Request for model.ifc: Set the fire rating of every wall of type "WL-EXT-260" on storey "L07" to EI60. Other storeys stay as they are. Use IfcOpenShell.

First a look at what the model holds.

```python
import ifcopenshell
import ifcopenshell.util.element

model = ifcopenshell.open("model.ifc")
print(model.schema)
storey = next(s for s in model.by_type("IfcBuildingStorey") if s.Name == "L07")
walls = [e for e in ifcopenshell.util.element.get_decomposition(storey) if e.is_a("IfcWall")]
seen = {}
for e in walls:
    element_type = ifcopenshell.util.element.get_type(e)
    key = (element_type.Name if element_type != e and element_type else None, ifcopenshell.util.element.get_pset(e, "Pset_WallCommon", "FireRating"))
    seen[key] = seen.get(key, 0) + 1
for (name, value), count in sorted(seen.items(), key=str):
    print(count, "x", name, "|", value)
```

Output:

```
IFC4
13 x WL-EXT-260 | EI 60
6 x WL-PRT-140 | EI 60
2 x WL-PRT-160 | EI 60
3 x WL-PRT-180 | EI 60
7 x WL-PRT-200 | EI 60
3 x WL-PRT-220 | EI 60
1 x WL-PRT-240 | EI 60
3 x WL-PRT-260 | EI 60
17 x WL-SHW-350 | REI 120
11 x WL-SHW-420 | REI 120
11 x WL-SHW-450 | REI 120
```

```python
import ifcopenshell
import ifcopenshell.api.pset
import ifcopenshell.util.element

model = ifcopenshell.open("model.ifc")

storey = next(s for s in model.by_type("IfcBuildingStorey") if s.Name == "L07")
walls = [e for e in ifcopenshell.util.element.get_decomposition(storey) if e.is_a("IfcWall")]

count = 0
for e in walls:
    element_type = ifcopenshell.util.element.get_type(e)
    if element_type in (None, e) or element_type.Name != "WL-EXT-260":
        continue
    # add_pset returns the element's existing set when there is one.
    pset = ifcopenshell.api.pset.add_pset(model, product=e, name="Pset_WallCommon")
    ifcopenshell.api.pset.edit_pset(model, pset=pset, properties={"FireRating": "EI60"})
    count += 1

print(count, "walls updated")

model.write("model-out.ifc")
```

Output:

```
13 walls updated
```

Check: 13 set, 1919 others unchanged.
